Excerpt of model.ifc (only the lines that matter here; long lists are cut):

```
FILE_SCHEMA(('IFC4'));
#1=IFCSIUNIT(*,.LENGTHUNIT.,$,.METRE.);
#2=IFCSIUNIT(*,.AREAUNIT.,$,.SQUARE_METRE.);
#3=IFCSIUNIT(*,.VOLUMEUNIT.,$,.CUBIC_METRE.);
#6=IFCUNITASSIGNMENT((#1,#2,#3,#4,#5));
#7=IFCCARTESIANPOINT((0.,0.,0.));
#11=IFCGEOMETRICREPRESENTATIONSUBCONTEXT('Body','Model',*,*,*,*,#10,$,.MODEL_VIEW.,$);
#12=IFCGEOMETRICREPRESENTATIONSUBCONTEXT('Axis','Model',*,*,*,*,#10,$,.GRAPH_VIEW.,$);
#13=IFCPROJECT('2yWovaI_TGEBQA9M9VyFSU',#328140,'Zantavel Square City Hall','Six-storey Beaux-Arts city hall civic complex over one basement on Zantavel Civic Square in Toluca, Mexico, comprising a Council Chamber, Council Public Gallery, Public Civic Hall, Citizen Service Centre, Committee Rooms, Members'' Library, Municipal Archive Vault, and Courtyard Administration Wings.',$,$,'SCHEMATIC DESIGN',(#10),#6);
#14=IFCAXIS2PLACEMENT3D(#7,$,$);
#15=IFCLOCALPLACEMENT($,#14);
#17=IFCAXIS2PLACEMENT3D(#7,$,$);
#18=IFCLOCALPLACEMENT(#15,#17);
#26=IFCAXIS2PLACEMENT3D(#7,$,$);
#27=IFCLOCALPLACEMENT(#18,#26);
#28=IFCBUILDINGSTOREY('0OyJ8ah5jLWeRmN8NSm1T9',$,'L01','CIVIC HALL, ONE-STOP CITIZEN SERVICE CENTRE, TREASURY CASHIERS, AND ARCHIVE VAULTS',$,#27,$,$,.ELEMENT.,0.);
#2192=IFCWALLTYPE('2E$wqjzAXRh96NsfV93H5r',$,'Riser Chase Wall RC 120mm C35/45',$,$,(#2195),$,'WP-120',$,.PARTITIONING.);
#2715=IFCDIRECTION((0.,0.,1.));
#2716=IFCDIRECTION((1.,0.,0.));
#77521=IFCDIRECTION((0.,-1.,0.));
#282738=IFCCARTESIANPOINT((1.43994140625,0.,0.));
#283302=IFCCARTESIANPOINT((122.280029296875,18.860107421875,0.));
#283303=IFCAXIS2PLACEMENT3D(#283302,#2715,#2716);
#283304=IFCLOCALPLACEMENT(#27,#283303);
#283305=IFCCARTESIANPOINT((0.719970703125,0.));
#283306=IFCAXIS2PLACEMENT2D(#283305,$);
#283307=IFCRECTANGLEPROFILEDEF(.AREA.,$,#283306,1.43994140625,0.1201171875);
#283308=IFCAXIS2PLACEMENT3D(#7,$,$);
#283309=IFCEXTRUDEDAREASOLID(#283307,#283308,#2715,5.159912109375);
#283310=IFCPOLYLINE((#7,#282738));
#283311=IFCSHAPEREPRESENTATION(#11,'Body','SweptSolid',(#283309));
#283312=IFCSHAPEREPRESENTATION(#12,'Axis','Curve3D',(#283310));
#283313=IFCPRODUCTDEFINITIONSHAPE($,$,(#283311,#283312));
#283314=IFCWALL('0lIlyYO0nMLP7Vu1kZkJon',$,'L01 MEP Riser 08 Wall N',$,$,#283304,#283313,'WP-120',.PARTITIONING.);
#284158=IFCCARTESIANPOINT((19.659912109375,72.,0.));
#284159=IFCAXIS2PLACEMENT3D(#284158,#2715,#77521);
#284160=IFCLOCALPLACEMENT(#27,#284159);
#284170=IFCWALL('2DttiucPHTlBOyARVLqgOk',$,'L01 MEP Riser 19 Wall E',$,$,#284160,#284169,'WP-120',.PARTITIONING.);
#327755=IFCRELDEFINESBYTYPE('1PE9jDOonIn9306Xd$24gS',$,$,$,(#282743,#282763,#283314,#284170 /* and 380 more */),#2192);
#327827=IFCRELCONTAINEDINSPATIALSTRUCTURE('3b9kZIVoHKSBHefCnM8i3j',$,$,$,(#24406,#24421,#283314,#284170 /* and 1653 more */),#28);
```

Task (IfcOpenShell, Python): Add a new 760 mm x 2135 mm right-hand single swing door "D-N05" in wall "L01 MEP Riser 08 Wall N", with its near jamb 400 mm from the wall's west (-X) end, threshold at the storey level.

```python
import numpy as np
import ifcopenshell
import ifcopenshell.api.feature
import ifcopenshell.api.geometry
import ifcopenshell.api.root
import ifcopenshell.api.spatial
import ifcopenshell.geom
import ifcopenshell.util.element
import ifcopenshell.util.placement
import ifcopenshell.util.representation
import ifcopenshell.util.shape
import ifcopenshell.util.unit

model = ifcopenshell.open("model.ifc")
unit_scale = ifcopenshell.util.unit.calculate_unit_scale(model)
settings = ifcopenshell.geom.settings()


def volume(element):
    """Net volume in cubic metres, openings subtracted."""
    shape = ifcopenshell.geom.create_shape(settings, element)
    return ifcopenshell.util.shape.get_volume(shape.geometry)


wall = model.by_guid("0lIlyYO0nMLP7Vu1kZkJon")
storey = ifcopenshell.util.element.get_container(wall, ifc_class="IfcBuildingStorey")
context = ifcopenshell.util.representation.get_context(model, "Model", "Body", "MODEL_VIEW")
before = volume(wall)

width, height, from_end, sill = 0.76, 2.135, 0.4, 0.0  # metres

# The wall runs along its own X axis, and the end named is its -X end.
wall_shape = ifcopenshell.geom.create_shape(settings, wall)
x, y, z = ifcopenshell.util.shape.get_vertices(wall_shape.geometry).T
start = x.min() + from_end
face, thickness = float(y.min()), float(y.max() - y.min())
wall_matrix = ifcopenshell.util.placement.get_local_placement(wall.ObjectPlacement)
level = ifcopenshell.util.placement.get_local_placement(storey.ObjectPlacement)[2, 3]


def in_wall(x, y):
    """Placement at x, y metres in the wall's axes, at sill height."""
    matrix = wall_matrix.copy()
    matrix[:, 3] = wall_matrix @ np.array([x / unit_scale, y / unit_scale, 0.0, 1.0])
    matrix[2, 3] = level + sill / unit_scale
    return matrix


# Opening: a box that overshoots both wall faces by 50 mm.
opening = ifcopenshell.api.root.create_entity(model, ifc_class="IfcOpeningElement", predefined_type="OPENING")
box = ifcopenshell.api.geometry.add_wall_representation(
    model, context=context, length=width, height=height, thickness=thickness + 0.1
)
ifcopenshell.api.geometry.assign_representation(model, product=opening, representation=box)
ifcopenshell.api.geometry.edit_object_placement(model, product=opening, matrix=in_wall(start, face - 0.05), is_si=False)
ifcopenshell.api.feature.add_feature(model, feature=opening, element=wall)

door = ifcopenshell.api.root.create_entity(model, ifc_class="IfcDoor", name="D-N05", predefined_type="DOOR")
door.OverallWidth, door.OverallHeight = width / unit_scale, height / unit_scale
door.OperationType = "SINGLE_SWING_RIGHT"
body = ifcopenshell.api.geometry.add_door_representation(
    model,
    context=context,
    overall_width=door.OverallWidth,
    overall_height=door.OverallHeight,
    operation_type="SINGLE_SWING_RIGHT",
    lining_properties={"LiningDepth": thickness / unit_scale, "ThresholdDepth": thickness / unit_scale},
)
ifcopenshell.api.geometry.assign_representation(model, product=door, representation=body)
ifcopenshell.api.spatial.assign_container(model, products=[door], relating_structure=storey)
ifcopenshell.api.feature.add_filling(model, opening=opening, element=door)

# The lining spans the wall, so the door starts at the wall face.
ifcopenshell.api.geometry.edit_object_placement(model, product=door, matrix=in_wall(start, face), is_si=False)

after = volume(wall)

print(f"wall volume {before:.3f} -> {after:.3f} m3")

model.write("model-out.ifc")
```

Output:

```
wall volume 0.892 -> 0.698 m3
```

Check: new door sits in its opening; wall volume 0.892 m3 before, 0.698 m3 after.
